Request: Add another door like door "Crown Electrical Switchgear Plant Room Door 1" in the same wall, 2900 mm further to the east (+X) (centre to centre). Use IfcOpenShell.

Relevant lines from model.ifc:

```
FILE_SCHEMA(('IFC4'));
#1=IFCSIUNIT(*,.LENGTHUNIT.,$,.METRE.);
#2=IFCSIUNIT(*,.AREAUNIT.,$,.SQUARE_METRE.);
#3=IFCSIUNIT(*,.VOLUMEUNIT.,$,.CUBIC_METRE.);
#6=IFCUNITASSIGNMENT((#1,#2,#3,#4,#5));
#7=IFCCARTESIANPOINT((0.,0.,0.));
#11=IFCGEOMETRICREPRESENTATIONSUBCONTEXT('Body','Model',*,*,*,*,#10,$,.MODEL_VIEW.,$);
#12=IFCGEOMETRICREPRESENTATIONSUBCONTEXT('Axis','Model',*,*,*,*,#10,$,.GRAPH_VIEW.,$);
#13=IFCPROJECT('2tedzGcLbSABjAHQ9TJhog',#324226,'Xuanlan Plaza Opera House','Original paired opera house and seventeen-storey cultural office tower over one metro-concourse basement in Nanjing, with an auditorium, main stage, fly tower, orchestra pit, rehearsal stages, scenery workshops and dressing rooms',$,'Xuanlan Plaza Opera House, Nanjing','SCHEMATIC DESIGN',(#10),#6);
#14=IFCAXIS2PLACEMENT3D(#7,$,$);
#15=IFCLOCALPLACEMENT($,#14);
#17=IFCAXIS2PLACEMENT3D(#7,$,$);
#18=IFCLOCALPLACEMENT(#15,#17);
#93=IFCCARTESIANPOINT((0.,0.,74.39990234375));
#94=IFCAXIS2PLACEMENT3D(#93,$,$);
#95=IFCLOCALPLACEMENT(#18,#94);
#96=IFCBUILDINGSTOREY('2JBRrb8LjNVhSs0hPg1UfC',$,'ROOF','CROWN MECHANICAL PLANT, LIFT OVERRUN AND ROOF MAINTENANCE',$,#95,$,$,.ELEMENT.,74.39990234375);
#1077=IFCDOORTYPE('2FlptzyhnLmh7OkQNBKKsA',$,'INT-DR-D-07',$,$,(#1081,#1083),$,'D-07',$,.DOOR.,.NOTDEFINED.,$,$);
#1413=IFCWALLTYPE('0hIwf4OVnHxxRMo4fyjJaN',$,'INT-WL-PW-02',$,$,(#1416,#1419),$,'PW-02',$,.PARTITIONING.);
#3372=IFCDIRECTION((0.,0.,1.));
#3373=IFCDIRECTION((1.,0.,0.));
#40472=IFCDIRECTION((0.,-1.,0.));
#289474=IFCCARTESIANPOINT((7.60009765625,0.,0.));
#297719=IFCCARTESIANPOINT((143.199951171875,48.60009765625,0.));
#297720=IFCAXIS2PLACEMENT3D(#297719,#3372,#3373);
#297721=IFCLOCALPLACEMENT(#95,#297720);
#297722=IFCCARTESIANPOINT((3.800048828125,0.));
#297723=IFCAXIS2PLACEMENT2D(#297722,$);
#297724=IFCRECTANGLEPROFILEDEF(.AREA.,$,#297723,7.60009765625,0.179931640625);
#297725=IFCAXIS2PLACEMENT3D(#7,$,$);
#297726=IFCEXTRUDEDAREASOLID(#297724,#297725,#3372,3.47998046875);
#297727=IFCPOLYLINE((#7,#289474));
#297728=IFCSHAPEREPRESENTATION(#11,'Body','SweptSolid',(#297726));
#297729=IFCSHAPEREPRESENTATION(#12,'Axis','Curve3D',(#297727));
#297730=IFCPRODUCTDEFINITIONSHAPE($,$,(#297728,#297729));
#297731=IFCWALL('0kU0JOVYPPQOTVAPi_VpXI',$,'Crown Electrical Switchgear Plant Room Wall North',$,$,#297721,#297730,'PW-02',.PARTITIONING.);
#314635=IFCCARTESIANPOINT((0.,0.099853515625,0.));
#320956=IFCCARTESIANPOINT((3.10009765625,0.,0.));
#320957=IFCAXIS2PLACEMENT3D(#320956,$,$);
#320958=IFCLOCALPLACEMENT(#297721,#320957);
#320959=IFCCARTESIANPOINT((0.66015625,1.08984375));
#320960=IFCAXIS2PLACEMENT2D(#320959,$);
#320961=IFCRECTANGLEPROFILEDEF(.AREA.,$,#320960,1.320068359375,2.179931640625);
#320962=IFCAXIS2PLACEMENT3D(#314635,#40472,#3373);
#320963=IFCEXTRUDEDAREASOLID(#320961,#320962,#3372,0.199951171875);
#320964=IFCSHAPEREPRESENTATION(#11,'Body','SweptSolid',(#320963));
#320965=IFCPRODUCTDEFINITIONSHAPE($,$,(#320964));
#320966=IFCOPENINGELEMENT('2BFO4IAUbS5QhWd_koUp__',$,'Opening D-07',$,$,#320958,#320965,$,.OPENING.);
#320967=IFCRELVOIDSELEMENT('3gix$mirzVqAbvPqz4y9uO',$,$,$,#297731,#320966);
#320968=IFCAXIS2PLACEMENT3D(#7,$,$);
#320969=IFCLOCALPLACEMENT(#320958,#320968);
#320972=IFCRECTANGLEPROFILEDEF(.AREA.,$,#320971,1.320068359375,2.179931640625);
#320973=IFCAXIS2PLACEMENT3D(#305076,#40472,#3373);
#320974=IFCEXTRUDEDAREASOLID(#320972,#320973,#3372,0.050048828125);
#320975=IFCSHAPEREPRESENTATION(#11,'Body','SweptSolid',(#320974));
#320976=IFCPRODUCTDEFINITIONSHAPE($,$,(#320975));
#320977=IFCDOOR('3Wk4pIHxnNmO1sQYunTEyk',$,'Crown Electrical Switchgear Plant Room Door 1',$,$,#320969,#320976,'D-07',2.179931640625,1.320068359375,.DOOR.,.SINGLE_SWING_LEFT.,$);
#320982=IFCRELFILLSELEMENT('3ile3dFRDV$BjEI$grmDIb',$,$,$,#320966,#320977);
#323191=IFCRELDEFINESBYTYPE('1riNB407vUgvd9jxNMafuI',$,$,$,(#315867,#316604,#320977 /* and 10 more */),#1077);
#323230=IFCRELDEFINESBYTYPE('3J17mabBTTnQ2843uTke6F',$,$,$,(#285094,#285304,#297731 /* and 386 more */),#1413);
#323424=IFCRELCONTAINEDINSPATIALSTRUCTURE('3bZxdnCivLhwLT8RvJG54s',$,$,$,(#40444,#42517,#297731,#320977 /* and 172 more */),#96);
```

```python
import ifcopenshell
import ifcopenshell.api.feature
import ifcopenshell.api.geometry
import ifcopenshell.api.root
import ifcopenshell.geom
import ifcopenshell.util.element
import ifcopenshell.util.placement
import ifcopenshell.util.shape

model = ifcopenshell.open("model.ifc")
settings = ifcopenshell.geom.settings()


def volume(element):
    """Net volume in cubic metres, openings subtracted."""
    shape = ifcopenshell.geom.create_shape(settings, element)
    return ifcopenshell.util.shape.get_volume(shape.geometry)


door = model.by_guid("3Wk4pIHxnNmO1sQYunTEyk")
opening = door.FillsVoids[0].RelatingOpeningElement
wall = opening.VoidsElements[0].RelatingBuildingElement
before = volume(wall)
shift = ifcopenshell.util.placement.get_local_placement(wall.ObjectPlacement)[:3, 0] * 2.9

# copy_class copies the void relationship, type, container and properties, but no geometry.
new_opening = ifcopenshell.api.root.copy_class(model, product=opening)
new_opening.Representation = ifcopenshell.util.element.copy_deep(
    model, opening.Representation, exclude=["IfcGeometricRepresentationContext", "IfcRepresentationMap"]
)
new_door = ifcopenshell.api.root.copy_class(model, product=door)
new_door.Representation = ifcopenshell.util.element.copy_deep(
    model, door.Representation, exclude=["IfcGeometricRepresentationContext", "IfcRepresentationMap"]
)
new_door.Tag = None
ifcopenshell.api.feature.add_filling(model, opening=new_opening, element=new_door)

for old, new in ((opening, new_opening), (door, new_door)):
    matrix = ifcopenshell.util.placement.get_local_placement(old.ObjectPlacement)
    matrix[:3, 3] += shift
    ifcopenshell.api.geometry.edit_object_placement(model, product=new, matrix=matrix, is_si=False)

after = volume(wall)

print(f"wall volume {before:.3f} -> {after:.3f} m3")

model.write("model_edited.ifc")
```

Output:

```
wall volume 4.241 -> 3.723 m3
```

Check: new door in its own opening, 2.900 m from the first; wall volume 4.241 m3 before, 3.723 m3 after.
